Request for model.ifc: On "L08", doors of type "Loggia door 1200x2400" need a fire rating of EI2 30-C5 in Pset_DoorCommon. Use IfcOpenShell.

First a look at what the model holds.

```python
import ifcopenshell
import ifcopenshell.util.element

model = ifcopenshell.open("model.ifc")
print(model.schema)
storey = next(s for s in model.by_type("IfcBuildingStorey") if s.Name == "L08")
doors = [e for e in ifcopenshell.util.element.get_decomposition(storey) if e.is_a("IfcDoor")]
seen = {}
for e in doors:
    element_type = ifcopenshell.util.element.get_type(e)
    key = (element_type.Name if element_type != e and element_type else None, ifcopenshell.util.element.get_pset(e, "Pset_DoorCommon", "FireRating"))
    seen[key] = seen.get(key, 0) + 1
for (name, value), count in sorted(seen.items(), key=str):
    print(count, "x", name, "|", value)
```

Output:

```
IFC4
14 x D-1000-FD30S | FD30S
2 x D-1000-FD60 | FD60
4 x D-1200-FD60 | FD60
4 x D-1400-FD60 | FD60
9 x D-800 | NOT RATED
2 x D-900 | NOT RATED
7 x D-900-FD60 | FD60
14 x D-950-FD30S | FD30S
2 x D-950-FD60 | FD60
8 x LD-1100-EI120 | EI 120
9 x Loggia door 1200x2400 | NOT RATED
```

```python
import ifcopenshell
import ifcopenshell.api.pset
import ifcopenshell.util.element

model = ifcopenshell.open("model.ifc")

storey = next(s for s in model.by_type("IfcBuildingStorey") if s.Name == "L08")
doors = [e for e in ifcopenshell.util.element.get_decomposition(storey) if e.is_a("IfcDoor")]

count = 0
for e in doors:
    element_type = ifcopenshell.util.element.get_type(e)
    if element_type in (None, e) or element_type.Name != "Loggia door 1200x2400":
        continue
    # add_pset returns the element's existing set when there is one.
    pset = ifcopenshell.api.pset.add_pset(model, product=e, name="Pset_DoorCommon")
    ifcopenshell.api.pset.edit_pset(model, pset=pset, properties={"FireRating": "EI2 30-C5"})
    count += 1

print(count, "doors updated")

model.write("model_v2.ifc")
```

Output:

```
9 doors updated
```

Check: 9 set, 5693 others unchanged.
